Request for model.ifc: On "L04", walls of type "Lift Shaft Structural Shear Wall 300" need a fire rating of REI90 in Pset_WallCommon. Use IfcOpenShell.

First a look at what the model holds.

```python
import ifcopenshell
import ifcopenshell.util.element

model = ifcopenshell.open("model.ifc")
print(model.schema)
storey = next(s for s in model.by_type("IfcBuildingStorey") if s.Name == "L04")
walls = [e for e in ifcopenshell.util.element.get_decomposition(storey) if e.is_a("IfcWall")]
seen = {}
for e in walls:
    element_type = ifcopenshell.util.element.get_type(e)
    key = (element_type.Name if element_type != e and element_type else None, ifcopenshell.util.element.get_pset(e, "Pset_WallCommon", "FireRating"))
    seen[key] = seen.get(key, 0) + 1
for (name, value), count in sorted(seen.items(), key=str):
    print(count, "x", name, "|", value)
```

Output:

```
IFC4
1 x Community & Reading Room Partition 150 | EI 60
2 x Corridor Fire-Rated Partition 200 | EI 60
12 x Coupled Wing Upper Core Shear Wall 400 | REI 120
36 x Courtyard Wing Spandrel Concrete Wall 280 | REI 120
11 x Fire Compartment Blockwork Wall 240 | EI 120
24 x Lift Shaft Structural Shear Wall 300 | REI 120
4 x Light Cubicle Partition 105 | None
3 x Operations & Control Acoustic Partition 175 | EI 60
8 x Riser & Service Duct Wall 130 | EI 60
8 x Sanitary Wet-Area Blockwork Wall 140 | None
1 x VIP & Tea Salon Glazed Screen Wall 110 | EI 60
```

```python
import ifcopenshell
import ifcopenshell.api.pset
import ifcopenshell.util.element

model = ifcopenshell.open("model.ifc")

storey = next(s for s in model.by_type("IfcBuildingStorey") if s.Name == "L04")
walls = [e for e in ifcopenshell.util.element.get_decomposition(storey) if e.is_a("IfcWall")]

count = 0
for e in walls:
    element_type = ifcopenshell.util.element.get_type(e)
    if element_type in (None, e) or element_type.Name != "Lift Shaft Structural Shear Wall 300":
        continue
    # add_pset returns the element's existing set when there is one.
    pset = ifcopenshell.api.pset.add_pset(model, product=e, name="Pset_WallCommon")
    ifcopenshell.api.pset.edit_pset(model, pset=pset, properties={"FireRating": "REI90"})
    count += 1

print(count, "walls updated")

model.write("model_updated.ifc")
```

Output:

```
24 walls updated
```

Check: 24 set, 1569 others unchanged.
